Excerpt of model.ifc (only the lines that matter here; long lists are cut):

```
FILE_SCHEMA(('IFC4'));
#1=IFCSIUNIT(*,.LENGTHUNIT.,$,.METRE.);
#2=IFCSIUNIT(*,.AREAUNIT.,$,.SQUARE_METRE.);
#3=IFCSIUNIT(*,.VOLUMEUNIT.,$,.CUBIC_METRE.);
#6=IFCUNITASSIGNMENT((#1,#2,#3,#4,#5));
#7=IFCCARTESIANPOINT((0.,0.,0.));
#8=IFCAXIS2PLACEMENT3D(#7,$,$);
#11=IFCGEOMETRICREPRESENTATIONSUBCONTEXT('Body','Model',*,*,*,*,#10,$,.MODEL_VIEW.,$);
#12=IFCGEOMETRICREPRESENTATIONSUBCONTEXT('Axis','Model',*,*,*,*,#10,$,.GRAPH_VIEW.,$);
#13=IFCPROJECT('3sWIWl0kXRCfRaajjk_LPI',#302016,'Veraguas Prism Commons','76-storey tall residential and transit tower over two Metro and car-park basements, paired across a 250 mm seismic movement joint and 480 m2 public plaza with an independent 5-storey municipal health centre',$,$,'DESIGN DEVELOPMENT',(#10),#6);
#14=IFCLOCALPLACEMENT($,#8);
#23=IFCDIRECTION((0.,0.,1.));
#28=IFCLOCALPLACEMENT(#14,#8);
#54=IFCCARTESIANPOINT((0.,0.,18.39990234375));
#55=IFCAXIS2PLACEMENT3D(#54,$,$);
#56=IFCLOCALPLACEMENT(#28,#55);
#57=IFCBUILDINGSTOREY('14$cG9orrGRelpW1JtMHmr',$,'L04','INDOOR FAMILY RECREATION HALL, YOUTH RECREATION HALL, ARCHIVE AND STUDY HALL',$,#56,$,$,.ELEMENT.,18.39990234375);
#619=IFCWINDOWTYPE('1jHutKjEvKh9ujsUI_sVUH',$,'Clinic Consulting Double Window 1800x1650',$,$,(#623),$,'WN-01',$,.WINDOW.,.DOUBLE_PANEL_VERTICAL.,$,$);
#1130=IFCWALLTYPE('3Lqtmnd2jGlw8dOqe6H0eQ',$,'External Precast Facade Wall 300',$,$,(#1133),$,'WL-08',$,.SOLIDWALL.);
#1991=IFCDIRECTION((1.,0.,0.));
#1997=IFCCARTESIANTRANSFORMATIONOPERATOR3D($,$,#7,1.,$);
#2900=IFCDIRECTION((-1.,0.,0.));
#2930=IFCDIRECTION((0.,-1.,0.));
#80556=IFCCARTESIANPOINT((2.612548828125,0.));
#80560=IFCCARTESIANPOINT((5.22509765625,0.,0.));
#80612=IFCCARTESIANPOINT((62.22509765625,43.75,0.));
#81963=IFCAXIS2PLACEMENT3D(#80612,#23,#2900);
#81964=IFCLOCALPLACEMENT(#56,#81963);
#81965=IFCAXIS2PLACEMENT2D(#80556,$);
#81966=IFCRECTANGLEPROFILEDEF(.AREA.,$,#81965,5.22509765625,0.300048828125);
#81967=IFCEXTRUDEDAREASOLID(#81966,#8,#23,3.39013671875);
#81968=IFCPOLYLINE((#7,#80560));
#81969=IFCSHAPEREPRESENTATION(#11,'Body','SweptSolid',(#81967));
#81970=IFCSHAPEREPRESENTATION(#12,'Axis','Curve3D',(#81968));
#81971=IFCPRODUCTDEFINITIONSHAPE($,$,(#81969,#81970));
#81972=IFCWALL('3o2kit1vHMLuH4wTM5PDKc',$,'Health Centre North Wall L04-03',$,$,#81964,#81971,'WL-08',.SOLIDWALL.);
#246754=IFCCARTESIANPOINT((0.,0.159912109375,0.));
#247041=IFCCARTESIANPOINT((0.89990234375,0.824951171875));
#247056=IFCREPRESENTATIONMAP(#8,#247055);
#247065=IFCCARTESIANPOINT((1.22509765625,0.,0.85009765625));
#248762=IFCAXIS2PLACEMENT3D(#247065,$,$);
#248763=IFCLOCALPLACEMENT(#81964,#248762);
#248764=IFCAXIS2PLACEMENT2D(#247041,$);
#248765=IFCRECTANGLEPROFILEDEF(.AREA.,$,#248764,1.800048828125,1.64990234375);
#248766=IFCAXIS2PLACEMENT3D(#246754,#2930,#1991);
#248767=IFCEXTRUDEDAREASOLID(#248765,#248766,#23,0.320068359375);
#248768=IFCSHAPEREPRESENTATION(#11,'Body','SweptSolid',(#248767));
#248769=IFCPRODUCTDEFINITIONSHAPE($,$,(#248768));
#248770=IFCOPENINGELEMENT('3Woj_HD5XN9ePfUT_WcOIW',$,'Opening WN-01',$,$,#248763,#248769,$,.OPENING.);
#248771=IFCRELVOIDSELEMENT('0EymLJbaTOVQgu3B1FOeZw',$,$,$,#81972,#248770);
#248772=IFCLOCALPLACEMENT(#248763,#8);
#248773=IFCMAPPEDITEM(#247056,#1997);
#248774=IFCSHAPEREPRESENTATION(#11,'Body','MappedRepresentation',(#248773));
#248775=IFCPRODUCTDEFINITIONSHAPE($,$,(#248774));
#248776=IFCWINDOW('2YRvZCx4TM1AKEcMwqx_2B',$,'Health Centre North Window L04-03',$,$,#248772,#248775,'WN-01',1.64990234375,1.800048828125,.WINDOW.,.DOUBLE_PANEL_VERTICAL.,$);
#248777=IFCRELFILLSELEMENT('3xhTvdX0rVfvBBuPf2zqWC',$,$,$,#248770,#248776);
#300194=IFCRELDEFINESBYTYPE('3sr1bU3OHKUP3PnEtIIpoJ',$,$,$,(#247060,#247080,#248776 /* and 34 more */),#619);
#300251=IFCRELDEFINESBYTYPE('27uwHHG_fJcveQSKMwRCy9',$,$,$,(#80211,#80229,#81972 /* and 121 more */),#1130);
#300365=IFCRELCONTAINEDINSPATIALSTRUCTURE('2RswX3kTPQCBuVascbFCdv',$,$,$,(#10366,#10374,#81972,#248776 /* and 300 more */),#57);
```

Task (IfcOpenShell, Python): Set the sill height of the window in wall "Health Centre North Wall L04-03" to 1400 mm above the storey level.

```python
import numpy as np
import ifcopenshell
import ifcopenshell.api.geometry
import ifcopenshell.geom
import ifcopenshell.util.element
import ifcopenshell.util.placement
import ifcopenshell.util.shape
import ifcopenshell.util.unit

model = ifcopenshell.open("model.ifc")
unit_scale = ifcopenshell.util.unit.calculate_unit_scale(model)

window = model.by_id(248776)
opening = window.FillsVoids[0].RelatingOpeningElement
storey = ifcopenshell.util.element.get_container(window, ifc_class="IfcBuildingStorey")
level = ifcopenshell.util.placement.get_local_placement(storey.ObjectPlacement)[2, 3]

# The opening's origin need not be at the sill, so measure its lowest point.
shape = ifcopenshell.geom.create_shape(ifcopenshell.geom.settings(), opening)
bottom = ifcopenshell.util.shape.get_shape_bottom_elevation(shape, shape.geometry) / unit_scale
dz = level + 1.4 - bottom

shift = np.array([0.0, 0.0, dz])
# The window is placed relative to its opening, so it follows when the opening moves.
matrix = ifcopenshell.util.placement.get_local_placement(opening.ObjectPlacement)
matrix[:3, 3] += shift
ifcopenshell.api.geometry.edit_object_placement(
    model, product=opening, matrix=matrix, is_si=False, should_transform_children=True
)

print(f"moved by {dz * unit_scale:+.3f} m")

model.write("model_updated.ifc")
```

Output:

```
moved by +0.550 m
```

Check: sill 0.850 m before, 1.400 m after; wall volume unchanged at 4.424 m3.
